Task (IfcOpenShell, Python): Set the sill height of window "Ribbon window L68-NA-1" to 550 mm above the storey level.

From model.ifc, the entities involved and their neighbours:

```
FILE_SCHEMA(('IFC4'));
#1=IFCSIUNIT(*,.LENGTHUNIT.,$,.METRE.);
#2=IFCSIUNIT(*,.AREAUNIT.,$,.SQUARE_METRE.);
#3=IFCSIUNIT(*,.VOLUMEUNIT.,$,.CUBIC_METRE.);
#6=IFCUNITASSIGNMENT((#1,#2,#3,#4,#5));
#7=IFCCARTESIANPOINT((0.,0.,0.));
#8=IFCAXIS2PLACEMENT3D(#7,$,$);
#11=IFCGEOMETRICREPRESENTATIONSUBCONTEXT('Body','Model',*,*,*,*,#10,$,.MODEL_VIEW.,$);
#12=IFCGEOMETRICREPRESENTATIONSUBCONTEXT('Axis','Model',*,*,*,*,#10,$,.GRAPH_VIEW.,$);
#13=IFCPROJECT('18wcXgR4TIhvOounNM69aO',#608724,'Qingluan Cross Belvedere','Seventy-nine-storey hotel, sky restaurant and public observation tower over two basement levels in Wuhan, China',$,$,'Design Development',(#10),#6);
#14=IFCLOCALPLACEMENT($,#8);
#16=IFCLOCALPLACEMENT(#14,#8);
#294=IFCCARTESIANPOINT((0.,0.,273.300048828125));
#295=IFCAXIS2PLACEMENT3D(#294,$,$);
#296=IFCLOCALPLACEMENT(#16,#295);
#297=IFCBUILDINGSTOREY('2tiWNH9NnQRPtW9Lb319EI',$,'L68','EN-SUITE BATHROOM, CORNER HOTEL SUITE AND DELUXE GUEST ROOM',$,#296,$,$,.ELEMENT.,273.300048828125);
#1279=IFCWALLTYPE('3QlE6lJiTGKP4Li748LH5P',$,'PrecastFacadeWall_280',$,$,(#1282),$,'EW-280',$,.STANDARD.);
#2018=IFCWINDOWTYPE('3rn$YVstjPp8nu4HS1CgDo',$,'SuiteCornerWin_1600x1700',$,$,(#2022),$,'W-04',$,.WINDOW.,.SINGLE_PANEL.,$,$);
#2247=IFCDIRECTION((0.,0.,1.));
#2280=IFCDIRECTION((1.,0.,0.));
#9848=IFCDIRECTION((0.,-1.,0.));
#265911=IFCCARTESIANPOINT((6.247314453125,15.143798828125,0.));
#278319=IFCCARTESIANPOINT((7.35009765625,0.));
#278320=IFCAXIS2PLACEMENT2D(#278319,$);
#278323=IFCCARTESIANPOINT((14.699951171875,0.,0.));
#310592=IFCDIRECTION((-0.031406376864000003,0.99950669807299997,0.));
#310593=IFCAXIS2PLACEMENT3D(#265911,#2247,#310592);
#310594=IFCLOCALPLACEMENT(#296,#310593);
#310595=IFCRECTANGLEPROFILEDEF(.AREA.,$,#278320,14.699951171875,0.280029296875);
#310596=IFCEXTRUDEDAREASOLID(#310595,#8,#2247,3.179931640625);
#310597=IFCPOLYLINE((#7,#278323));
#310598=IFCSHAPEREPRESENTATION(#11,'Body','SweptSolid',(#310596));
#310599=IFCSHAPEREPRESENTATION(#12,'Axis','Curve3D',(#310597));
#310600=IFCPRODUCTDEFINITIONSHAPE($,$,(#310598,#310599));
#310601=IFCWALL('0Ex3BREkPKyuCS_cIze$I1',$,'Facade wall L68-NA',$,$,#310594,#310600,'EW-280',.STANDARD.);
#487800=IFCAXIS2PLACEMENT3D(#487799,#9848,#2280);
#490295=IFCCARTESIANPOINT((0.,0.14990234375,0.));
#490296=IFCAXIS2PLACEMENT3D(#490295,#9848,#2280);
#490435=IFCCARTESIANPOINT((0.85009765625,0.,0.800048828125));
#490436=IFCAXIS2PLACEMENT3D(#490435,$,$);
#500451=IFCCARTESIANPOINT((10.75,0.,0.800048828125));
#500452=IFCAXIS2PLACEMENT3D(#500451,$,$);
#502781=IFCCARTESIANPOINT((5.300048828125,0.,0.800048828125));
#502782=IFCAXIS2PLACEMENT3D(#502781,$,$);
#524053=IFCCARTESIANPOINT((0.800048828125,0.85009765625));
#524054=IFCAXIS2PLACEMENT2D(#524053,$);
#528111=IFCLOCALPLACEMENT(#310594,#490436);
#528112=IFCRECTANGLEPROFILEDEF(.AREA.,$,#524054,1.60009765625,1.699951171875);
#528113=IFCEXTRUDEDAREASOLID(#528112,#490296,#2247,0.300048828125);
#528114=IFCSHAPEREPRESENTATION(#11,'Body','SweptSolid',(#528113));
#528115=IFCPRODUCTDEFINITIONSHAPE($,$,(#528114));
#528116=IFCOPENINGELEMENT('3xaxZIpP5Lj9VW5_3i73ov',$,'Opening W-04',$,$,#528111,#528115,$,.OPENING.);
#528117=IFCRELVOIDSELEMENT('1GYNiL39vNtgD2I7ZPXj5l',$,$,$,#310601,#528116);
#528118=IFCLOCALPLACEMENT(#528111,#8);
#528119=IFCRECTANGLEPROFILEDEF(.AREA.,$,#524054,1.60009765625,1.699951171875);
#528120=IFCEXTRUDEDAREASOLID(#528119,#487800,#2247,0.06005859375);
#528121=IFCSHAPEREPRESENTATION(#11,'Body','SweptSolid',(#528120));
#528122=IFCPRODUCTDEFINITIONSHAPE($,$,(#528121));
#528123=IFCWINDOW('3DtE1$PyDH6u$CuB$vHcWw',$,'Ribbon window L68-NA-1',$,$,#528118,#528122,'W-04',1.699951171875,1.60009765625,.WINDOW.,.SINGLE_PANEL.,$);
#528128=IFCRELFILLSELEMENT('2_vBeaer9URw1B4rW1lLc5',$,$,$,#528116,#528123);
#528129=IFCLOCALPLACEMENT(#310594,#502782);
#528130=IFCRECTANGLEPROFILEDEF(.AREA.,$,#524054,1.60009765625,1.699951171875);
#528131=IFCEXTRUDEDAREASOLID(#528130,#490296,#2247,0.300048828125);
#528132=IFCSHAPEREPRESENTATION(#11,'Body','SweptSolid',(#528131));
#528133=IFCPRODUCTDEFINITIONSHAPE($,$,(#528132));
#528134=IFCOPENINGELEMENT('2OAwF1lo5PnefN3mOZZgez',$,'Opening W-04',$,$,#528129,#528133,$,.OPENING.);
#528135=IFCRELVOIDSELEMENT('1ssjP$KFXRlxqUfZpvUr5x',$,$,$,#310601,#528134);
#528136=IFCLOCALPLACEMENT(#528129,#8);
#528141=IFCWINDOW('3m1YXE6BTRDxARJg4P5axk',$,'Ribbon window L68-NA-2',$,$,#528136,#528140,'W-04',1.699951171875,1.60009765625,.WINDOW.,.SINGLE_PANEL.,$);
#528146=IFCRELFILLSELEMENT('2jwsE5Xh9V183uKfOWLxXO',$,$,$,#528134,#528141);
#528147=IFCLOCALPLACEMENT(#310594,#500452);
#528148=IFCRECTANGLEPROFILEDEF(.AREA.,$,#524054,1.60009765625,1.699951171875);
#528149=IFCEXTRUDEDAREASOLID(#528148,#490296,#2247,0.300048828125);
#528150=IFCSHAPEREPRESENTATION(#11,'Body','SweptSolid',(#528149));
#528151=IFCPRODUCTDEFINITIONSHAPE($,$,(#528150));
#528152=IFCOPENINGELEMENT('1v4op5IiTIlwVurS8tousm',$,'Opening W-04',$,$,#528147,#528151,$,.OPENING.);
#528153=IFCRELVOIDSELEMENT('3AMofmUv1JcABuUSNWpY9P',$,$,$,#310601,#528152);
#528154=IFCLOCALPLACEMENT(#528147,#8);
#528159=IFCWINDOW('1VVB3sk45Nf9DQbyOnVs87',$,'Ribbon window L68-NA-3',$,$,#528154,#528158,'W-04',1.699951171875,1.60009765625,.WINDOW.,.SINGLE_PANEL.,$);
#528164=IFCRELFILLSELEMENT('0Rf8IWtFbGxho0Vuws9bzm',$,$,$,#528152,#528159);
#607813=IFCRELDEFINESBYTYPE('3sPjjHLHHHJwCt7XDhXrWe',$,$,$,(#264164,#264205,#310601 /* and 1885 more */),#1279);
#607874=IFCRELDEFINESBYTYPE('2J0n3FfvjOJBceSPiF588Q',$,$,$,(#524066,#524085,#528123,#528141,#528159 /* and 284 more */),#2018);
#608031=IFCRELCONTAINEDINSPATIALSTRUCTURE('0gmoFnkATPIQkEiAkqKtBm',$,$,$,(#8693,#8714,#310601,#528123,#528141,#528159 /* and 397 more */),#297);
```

```python
import numpy as np
import ifcopenshell
import ifcopenshell.api.geometry
import ifcopenshell.geom
import ifcopenshell.util.element
import ifcopenshell.util.placement
import ifcopenshell.util.shape
import ifcopenshell.util.unit

model = ifcopenshell.open("model.ifc")
unit_scale = ifcopenshell.util.unit.calculate_unit_scale(model)

window = model.by_id(528123)
opening = window.FillsVoids[0].RelatingOpeningElement
storey = ifcopenshell.util.element.get_container(window, ifc_class="IfcBuildingStorey")
level = ifcopenshell.util.placement.get_local_placement(storey.ObjectPlacement)[2, 3]

# The opening's origin need not be at the sill, so measure its lowest point.
shape = ifcopenshell.geom.create_shape(ifcopenshell.geom.settings(), opening)
bottom = ifcopenshell.util.shape.get_shape_bottom_elevation(shape, shape.geometry) / unit_scale
dz = level + 0.55 - bottom

shift = np.array([0.0, 0.0, dz])
# The window is placed relative to its opening, so it follows when the opening moves.
matrix = ifcopenshell.util.placement.get_local_placement(opening.ObjectPlacement)
matrix[:3, 3] += shift
ifcopenshell.api.geometry.edit_object_placement(
    model, product=opening, matrix=matrix, is_si=False, should_transform_children=True
)

print(f"moved by {dz * unit_scale:+.3f} m")

model.write("model_v2.ifc")
```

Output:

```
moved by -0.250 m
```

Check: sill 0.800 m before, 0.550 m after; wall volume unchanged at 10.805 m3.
